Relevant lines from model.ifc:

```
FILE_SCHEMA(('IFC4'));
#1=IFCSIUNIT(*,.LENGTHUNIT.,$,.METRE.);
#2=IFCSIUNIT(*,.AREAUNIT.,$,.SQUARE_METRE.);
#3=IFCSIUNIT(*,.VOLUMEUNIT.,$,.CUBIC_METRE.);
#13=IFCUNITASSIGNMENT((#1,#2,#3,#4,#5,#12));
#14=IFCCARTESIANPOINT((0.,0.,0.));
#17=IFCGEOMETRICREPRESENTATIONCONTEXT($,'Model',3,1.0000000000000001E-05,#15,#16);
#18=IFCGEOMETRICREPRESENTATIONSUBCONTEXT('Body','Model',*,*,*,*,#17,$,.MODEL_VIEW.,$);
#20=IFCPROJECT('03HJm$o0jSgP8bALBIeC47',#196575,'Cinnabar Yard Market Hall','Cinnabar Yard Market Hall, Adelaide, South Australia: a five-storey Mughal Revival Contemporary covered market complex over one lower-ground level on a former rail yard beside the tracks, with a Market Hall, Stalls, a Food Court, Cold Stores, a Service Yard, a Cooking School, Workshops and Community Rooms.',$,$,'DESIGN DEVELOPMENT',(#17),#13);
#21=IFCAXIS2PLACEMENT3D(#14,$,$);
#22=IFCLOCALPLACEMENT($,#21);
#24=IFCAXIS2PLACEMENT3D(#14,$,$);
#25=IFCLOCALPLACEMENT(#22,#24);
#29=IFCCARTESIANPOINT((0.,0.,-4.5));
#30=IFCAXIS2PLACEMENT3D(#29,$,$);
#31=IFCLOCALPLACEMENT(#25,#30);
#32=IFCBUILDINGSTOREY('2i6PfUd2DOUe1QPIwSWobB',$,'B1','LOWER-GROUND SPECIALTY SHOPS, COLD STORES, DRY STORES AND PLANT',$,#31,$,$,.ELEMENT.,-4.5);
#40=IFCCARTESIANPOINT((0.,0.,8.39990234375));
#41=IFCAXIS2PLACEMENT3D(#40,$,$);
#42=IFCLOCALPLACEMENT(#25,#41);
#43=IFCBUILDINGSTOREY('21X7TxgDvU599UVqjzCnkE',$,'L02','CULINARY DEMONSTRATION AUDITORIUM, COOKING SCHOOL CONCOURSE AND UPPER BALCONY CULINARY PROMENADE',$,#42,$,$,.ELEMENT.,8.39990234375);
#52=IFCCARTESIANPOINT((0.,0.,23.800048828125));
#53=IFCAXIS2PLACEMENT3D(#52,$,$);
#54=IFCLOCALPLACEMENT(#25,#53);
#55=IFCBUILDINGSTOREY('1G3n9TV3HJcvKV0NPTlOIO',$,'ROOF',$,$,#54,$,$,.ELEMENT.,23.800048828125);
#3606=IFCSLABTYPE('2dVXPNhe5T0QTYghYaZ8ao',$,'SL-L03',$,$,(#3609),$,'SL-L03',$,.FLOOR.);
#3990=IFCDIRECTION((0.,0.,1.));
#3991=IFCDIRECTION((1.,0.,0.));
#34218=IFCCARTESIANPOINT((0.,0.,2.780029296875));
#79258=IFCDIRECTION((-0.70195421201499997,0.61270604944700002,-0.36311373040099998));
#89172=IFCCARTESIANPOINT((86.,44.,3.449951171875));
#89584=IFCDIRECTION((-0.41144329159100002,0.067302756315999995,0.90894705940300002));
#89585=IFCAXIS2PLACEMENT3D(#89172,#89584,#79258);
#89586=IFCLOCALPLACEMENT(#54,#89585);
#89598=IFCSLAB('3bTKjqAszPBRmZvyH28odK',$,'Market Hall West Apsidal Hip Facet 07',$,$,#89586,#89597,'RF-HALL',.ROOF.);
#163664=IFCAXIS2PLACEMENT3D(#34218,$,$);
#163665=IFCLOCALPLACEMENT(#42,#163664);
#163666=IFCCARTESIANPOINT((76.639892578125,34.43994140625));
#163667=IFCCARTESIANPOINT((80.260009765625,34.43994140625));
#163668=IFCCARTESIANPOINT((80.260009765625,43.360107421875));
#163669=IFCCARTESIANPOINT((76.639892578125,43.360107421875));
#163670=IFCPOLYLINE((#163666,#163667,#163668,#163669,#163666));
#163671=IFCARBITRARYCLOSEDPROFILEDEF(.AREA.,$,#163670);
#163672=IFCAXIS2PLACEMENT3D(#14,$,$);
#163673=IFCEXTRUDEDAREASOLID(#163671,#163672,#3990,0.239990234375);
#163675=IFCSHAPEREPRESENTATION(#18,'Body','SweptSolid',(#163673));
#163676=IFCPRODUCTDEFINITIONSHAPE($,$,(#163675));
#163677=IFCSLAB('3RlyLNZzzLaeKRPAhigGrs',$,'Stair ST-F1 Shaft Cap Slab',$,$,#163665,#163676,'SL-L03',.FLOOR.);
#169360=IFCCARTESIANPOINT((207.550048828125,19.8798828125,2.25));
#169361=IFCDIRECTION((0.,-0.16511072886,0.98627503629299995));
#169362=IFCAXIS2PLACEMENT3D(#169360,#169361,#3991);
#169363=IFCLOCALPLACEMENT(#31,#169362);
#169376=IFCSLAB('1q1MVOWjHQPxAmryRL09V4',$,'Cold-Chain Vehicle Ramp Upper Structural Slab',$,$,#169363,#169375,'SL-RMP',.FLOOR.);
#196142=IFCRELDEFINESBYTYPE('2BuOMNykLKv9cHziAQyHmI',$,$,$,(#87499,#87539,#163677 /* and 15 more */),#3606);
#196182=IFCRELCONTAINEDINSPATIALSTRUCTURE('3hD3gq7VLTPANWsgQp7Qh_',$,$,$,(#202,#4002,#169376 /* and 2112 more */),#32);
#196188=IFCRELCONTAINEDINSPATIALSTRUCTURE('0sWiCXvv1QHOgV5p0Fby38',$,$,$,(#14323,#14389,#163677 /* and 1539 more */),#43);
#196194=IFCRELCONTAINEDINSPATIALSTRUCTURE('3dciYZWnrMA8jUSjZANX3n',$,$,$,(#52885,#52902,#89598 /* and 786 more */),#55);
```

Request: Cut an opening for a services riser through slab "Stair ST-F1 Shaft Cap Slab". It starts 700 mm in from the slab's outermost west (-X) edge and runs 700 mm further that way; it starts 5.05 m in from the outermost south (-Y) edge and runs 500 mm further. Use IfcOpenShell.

```python
import numpy as np
import ifcopenshell
import ifcopenshell.api.feature
import ifcopenshell.api.geometry
import ifcopenshell.api.root
import ifcopenshell.geom
import ifcopenshell.util.placement
import ifcopenshell.util.representation
import ifcopenshell.util.shape
import ifcopenshell.util.unit

model = ifcopenshell.open("model.ifc")
unit_scale = ifcopenshell.util.unit.calculate_unit_scale(model)
settings = ifcopenshell.geom.settings()


def volume(element):
    """Net volume in cubic metres, openings subtracted."""
    shape = ifcopenshell.geom.create_shape(settings, element)
    return ifcopenshell.util.shape.get_volume(shape.geometry)


slab = model.by_guid("3RlyLNZzzLaeKRPAhigGrs")
before = volume(slab)

# Extent in the slab's own axes, in metres. The edges named are its -X and -Y sides.
slab_shape = ifcopenshell.geom.create_shape(settings, slab)
vertices = ifcopenshell.util.shape.get_vertices(slab_shape.geometry)
x_min, y_min, bottom = vertices.min(axis=0)
top = vertices[:, 2].max()

opening = ifcopenshell.api.root.create_entity(model, ifc_class="IfcOpeningElement", name="Services riser opening", predefined_type="OPENING")
context = ifcopenshell.util.representation.get_context(model, "Model", "Body", "MODEL_VIEW")
width, depth = 0.7, 0.5
outline = [(0.0, 0.0), (width, 0.0), (width, depth), (0.0, depth), (0.0, 0.0)]
# Overshoot both faces by 50 mm so the cut is clean.
shape = ifcopenshell.api.geometry.add_slab_representation(
    model, context=context, depth=top - bottom + 0.1, polyline=outline
)
ifcopenshell.api.geometry.assign_representation(model, product=opening, representation=shape)

matrix = ifcopenshell.util.placement.get_local_placement(slab.ObjectPlacement)
matrix[:, 3] = matrix @ np.append(np.array([x_min + 0.7, y_min + 5.05, bottom - 0.05]) / unit_scale, 1.0)
ifcopenshell.api.geometry.edit_object_placement(model, product=opening, matrix=matrix, is_si=False)
ifcopenshell.api.feature.add_feature(model, feature=opening, element=slab)

after = volume(slab)

print(f"slab volume {before:.3f} -> {after:.3f} m3")

model.write("model_v2.ifc")
```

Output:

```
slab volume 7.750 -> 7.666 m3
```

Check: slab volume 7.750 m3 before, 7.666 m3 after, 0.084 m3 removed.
